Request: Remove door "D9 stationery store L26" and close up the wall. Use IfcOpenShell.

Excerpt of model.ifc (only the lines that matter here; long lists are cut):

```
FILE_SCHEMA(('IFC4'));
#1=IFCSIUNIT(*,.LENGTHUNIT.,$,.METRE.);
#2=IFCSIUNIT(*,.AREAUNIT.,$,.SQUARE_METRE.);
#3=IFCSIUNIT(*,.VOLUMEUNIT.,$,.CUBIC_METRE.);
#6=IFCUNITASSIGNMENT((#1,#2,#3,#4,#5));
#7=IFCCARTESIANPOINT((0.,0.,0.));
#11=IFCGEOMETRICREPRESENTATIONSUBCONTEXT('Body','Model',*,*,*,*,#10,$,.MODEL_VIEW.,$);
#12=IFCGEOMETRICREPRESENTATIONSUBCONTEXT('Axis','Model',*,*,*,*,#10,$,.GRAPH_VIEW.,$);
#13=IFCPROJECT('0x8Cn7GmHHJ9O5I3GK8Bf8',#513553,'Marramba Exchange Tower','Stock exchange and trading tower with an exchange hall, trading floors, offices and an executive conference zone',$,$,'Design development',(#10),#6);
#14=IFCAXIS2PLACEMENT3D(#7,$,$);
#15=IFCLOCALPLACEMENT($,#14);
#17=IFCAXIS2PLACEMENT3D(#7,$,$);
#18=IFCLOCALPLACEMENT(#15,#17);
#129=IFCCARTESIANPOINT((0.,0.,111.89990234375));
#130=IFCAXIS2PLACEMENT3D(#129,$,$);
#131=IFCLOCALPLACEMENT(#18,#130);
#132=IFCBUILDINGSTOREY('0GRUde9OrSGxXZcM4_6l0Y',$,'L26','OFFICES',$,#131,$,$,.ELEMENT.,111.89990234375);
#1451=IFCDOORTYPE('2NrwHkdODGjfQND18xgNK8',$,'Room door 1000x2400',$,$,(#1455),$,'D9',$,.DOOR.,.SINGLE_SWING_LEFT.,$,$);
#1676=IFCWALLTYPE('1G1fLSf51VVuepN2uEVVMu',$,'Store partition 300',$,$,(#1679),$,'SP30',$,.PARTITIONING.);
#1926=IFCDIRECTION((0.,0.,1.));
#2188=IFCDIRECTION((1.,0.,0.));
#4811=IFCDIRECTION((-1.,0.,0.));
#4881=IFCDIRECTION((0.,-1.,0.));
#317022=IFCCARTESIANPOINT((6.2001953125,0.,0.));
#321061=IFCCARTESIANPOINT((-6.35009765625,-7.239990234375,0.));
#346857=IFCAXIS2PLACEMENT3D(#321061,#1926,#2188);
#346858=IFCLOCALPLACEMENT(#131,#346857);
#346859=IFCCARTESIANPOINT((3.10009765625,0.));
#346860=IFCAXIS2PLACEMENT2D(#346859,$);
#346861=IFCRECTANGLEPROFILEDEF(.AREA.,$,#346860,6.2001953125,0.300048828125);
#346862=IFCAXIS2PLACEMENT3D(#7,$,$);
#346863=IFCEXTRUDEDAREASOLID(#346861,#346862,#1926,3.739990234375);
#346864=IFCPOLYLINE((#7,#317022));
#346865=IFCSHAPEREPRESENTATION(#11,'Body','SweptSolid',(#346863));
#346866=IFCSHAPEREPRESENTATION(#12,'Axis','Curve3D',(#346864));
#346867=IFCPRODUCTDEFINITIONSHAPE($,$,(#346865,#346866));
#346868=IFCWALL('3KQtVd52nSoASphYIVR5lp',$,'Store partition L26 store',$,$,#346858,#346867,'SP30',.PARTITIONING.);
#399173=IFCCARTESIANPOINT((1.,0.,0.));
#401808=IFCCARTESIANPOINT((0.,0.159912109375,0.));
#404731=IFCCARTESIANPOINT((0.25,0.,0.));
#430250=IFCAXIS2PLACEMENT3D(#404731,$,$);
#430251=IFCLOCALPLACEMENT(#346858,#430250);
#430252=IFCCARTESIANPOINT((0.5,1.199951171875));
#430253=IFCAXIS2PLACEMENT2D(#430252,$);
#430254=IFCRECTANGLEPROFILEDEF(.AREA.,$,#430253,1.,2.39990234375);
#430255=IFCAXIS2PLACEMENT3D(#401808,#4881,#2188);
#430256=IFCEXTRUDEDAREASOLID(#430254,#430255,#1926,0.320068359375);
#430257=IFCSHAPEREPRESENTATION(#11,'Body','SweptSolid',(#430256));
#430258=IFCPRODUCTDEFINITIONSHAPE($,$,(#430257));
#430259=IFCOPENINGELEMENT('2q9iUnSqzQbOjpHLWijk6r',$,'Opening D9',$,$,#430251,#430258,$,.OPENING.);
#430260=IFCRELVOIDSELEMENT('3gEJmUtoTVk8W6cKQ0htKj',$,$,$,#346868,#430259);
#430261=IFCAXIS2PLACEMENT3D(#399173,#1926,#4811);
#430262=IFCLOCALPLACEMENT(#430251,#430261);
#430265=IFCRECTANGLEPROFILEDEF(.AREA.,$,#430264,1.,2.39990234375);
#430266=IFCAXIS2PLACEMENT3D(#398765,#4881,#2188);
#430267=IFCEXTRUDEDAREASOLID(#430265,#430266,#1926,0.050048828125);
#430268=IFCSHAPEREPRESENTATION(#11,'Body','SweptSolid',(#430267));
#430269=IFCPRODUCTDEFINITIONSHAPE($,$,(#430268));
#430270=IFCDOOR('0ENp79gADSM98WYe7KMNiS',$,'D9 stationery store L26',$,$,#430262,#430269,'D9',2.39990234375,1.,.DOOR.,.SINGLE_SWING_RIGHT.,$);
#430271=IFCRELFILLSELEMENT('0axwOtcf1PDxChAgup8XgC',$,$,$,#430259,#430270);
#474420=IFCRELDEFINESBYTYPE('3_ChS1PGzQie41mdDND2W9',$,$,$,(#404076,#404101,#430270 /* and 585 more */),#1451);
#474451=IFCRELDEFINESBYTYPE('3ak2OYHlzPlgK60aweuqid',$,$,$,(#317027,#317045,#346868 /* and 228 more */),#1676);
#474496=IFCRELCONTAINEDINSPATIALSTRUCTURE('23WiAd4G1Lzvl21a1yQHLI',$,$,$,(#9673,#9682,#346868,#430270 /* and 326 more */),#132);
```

```python
import ifcopenshell
import ifcopenshell.api.feature
import ifcopenshell.api.root
import ifcopenshell.geom
import ifcopenshell.util.shape

model = ifcopenshell.open("model.ifc")
settings = ifcopenshell.geom.settings()


def volume(element):
    """Net volume in cubic metres, openings subtracted."""
    shape = ifcopenshell.geom.create_shape(settings, element)
    return ifcopenshell.util.shape.get_volume(shape.geometry)


door = model.by_guid("0ENp79gADSM98WYe7KMNiS")
opening = door.FillsVoids[0].RelatingOpeningElement
wall = opening.VoidsElements[0].RelatingBuildingElement
before = volume(wall)

ifcopenshell.api.root.remove_product(model, product=door)
ifcopenshell.api.feature.remove_feature(model, feature=opening)

after = volume(wall)

print(f"wall volume {before:.3f} -> {after:.3f} m3")

model.write("model_rev.ifc")
```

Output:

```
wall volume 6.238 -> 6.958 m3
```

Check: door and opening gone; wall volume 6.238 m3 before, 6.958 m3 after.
